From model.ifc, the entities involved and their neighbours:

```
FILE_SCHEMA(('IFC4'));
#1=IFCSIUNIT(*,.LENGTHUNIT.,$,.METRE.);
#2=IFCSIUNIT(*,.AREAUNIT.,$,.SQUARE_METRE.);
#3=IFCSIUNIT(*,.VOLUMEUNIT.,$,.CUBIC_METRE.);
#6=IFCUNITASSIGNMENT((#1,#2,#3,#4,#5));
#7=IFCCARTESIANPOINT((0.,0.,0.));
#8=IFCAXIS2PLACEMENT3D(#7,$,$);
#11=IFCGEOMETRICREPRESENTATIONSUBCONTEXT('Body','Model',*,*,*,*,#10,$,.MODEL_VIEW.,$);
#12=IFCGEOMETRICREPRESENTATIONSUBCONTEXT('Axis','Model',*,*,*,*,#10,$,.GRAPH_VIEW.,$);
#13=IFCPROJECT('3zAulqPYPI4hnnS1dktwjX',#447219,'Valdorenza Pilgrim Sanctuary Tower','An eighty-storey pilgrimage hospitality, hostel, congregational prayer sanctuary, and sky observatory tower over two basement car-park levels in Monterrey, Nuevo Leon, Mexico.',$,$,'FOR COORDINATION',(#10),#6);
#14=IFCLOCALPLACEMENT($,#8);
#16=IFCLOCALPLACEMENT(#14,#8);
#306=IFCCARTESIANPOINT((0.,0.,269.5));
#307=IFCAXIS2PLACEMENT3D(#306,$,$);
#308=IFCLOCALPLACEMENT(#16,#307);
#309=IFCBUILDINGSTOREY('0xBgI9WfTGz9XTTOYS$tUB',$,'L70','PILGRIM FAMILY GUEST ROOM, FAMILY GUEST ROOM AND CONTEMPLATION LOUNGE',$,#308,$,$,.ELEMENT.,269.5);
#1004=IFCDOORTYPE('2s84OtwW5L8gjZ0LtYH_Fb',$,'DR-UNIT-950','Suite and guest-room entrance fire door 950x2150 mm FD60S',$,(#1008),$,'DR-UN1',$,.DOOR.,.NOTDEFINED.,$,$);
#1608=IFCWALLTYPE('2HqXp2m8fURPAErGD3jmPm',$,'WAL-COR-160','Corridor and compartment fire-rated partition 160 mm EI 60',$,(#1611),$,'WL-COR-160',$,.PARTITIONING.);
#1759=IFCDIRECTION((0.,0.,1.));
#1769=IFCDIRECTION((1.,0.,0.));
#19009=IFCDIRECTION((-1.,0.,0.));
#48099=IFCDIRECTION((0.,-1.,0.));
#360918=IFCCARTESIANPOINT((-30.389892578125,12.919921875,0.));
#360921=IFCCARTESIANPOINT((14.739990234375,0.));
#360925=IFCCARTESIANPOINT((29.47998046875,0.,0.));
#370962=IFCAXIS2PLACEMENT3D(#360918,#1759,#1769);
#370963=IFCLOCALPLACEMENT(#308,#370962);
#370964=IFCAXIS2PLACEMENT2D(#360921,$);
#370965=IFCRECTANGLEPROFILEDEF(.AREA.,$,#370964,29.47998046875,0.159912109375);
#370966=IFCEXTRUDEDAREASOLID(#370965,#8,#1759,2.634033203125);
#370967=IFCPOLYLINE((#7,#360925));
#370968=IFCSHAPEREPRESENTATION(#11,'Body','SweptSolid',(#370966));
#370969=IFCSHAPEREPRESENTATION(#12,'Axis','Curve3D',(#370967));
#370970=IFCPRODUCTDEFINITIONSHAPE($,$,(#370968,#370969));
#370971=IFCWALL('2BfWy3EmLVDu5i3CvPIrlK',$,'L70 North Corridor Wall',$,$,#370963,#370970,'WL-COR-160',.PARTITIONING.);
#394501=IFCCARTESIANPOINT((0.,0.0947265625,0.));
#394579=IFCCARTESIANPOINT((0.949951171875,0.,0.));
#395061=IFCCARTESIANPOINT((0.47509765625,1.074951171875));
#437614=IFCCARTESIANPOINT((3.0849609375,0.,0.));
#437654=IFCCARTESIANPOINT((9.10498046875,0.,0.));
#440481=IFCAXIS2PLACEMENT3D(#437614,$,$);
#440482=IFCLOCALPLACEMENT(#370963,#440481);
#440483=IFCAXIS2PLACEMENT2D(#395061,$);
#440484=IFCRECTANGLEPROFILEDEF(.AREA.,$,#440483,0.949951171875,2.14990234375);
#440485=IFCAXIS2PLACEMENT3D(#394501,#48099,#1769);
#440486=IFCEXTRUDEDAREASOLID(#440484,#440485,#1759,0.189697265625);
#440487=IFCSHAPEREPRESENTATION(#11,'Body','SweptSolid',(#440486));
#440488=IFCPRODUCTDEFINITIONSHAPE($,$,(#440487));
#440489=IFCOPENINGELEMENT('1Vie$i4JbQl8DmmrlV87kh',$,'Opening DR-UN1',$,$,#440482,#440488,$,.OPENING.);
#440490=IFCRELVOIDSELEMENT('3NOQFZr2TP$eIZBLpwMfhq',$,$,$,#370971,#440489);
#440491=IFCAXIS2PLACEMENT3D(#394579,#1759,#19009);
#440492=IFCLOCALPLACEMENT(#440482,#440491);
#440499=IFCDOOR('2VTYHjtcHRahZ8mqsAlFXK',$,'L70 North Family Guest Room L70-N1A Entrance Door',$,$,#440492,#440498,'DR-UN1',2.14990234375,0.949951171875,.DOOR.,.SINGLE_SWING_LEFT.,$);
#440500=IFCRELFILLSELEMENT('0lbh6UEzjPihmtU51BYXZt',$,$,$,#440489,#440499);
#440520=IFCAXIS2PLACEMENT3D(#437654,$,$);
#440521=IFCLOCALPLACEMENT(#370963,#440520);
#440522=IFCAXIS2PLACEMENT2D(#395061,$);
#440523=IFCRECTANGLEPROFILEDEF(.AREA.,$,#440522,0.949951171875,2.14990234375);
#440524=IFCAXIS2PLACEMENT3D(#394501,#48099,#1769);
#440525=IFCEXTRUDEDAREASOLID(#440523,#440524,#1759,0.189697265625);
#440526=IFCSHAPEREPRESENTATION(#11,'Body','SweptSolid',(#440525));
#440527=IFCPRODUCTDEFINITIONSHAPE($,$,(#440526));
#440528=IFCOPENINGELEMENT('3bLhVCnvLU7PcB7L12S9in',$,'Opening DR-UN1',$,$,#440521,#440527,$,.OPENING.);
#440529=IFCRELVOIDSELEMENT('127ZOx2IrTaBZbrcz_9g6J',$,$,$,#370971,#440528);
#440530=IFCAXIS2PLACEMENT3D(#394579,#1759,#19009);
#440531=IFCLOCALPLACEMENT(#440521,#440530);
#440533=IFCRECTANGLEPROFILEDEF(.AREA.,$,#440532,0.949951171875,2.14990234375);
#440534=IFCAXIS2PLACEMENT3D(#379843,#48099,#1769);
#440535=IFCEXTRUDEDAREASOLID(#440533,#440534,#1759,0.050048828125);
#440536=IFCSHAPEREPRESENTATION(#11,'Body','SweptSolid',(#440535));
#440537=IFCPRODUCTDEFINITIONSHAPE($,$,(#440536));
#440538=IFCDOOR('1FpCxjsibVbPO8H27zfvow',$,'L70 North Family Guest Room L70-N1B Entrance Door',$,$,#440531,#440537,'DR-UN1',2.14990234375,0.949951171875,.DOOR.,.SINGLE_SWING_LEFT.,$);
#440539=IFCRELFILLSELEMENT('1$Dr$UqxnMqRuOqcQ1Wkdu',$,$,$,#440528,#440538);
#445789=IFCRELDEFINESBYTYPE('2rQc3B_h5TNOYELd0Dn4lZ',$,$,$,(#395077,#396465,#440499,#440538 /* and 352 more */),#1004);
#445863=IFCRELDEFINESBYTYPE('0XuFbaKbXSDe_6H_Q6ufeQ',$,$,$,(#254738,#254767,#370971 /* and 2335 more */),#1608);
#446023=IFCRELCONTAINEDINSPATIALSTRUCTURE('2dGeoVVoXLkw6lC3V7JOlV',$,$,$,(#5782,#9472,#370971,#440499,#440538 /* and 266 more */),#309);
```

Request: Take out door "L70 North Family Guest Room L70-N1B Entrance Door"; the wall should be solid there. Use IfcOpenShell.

```python
import ifcopenshell
import ifcopenshell.api.feature
import ifcopenshell.api.root
import ifcopenshell.geom
import ifcopenshell.util.shape

model = ifcopenshell.open("model.ifc")
settings = ifcopenshell.geom.settings()


def volume(element):
    """Net volume in cubic metres, openings subtracted."""
    shape = ifcopenshell.geom.create_shape(settings, element)
    return ifcopenshell.util.shape.get_volume(shape.geometry)


door = model.by_id(440538)
opening = door.FillsVoids[0].RelatingOpeningElement
wall = opening.VoidsElements[0].RelatingBuildingElement
before = volume(wall)

ifcopenshell.api.root.remove_product(model, product=door)
ifcopenshell.api.feature.remove_feature(model, feature=opening)

after = volume(wall)

print(f"wall volume {before:.3f} -> {after:.3f} m3")

model.write("model_v2.ifc")
```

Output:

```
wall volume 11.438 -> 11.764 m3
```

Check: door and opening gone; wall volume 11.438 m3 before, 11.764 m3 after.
